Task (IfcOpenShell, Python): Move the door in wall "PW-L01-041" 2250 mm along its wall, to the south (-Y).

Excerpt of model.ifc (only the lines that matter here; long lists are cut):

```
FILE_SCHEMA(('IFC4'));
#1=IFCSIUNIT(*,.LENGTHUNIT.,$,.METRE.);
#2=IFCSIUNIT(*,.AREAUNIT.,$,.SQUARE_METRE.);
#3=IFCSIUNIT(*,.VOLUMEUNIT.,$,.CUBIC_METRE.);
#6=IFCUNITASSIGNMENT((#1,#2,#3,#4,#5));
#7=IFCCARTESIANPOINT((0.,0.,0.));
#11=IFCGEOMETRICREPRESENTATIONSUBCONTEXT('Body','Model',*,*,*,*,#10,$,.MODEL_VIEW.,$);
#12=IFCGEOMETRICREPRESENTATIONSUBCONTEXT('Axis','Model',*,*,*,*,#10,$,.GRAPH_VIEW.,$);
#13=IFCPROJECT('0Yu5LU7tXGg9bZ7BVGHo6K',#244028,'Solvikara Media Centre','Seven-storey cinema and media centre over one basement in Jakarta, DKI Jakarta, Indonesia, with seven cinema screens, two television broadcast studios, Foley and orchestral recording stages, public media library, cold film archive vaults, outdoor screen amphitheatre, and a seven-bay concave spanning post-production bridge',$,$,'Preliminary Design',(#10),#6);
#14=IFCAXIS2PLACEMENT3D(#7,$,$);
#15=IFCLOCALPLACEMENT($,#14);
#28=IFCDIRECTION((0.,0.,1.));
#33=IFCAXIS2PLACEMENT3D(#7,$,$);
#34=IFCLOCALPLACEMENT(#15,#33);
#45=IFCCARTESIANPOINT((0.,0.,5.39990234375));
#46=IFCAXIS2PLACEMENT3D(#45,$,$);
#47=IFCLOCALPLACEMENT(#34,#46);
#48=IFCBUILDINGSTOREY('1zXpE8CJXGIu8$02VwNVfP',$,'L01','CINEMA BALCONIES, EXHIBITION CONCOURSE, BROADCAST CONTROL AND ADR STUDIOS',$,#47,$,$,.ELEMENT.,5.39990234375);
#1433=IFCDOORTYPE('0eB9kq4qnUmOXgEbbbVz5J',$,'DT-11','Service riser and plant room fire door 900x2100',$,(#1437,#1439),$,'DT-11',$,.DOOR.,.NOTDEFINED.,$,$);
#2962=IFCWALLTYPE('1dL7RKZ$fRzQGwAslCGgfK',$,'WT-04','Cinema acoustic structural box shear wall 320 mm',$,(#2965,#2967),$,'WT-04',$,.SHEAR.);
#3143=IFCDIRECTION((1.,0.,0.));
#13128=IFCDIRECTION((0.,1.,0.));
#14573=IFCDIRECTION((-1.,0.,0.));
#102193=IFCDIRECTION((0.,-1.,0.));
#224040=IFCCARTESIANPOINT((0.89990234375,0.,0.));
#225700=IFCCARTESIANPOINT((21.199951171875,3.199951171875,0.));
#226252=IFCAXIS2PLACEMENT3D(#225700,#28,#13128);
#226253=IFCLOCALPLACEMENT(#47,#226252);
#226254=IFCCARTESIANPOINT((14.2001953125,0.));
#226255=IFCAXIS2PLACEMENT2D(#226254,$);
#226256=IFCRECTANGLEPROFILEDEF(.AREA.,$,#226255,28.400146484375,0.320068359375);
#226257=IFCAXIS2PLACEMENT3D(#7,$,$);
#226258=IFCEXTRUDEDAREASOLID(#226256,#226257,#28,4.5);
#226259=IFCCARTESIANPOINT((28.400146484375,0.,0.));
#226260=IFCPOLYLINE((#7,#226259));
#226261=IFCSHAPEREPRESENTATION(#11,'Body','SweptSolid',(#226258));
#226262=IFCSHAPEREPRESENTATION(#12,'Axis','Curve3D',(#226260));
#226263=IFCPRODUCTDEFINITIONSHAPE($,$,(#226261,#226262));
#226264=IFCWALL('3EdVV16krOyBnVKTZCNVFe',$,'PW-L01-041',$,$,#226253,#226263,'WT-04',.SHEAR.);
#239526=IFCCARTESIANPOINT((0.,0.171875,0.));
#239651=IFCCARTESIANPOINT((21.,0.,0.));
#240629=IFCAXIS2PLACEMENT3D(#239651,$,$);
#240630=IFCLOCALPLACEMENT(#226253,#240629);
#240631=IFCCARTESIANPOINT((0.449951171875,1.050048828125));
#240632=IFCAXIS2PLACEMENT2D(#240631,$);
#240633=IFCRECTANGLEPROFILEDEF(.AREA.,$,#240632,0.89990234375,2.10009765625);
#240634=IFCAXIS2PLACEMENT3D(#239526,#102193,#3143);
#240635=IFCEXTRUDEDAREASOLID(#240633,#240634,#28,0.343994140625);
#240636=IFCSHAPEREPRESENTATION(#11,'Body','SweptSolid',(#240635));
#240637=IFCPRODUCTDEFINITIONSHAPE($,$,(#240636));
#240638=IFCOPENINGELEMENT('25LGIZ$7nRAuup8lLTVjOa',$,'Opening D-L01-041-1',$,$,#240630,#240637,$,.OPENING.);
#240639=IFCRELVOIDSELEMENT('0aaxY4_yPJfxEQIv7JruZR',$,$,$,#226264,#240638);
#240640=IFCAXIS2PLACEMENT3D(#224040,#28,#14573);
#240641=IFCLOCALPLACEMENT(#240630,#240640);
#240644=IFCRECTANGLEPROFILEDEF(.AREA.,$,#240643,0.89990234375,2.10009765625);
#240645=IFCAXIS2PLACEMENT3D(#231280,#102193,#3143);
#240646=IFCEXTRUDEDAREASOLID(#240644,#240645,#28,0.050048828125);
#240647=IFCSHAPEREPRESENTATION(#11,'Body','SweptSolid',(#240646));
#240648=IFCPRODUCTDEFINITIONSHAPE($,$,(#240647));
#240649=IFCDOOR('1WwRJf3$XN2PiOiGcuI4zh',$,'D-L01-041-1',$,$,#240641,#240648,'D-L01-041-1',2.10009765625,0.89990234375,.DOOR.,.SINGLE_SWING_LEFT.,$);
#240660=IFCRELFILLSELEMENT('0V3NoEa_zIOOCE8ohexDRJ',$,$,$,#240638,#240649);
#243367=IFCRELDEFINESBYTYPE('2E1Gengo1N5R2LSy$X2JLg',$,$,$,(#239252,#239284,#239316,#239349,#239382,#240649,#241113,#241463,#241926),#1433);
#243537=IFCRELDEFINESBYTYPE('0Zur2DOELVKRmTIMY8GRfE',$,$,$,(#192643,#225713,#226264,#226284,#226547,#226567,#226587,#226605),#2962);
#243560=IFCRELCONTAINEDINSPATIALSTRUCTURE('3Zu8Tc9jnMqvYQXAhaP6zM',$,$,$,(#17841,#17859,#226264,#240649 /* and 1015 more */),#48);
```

```python
import ifcopenshell
import ifcopenshell.api.geometry
import ifcopenshell.util.placement

model = ifcopenshell.open("model.ifc")

door = model.by_guid("1WwRJf3$XN2PiOiGcuI4zh")
opening = door.FillsVoids[0].RelatingOpeningElement
wall = opening.VoidsElements[0].RelatingBuildingElement

wall_matrix = ifcopenshell.util.placement.get_local_placement(wall.ObjectPlacement)
shift = wall_matrix[:3, 0] * -2.25
before = ifcopenshell.util.placement.get_local_placement(door.ObjectPlacement)[:3, 3].copy()

# The door is placed relative to its opening, so it follows when the opening moves.
matrix = ifcopenshell.util.placement.get_local_placement(opening.ObjectPlacement)
matrix[:3, 3] += shift
ifcopenshell.api.geometry.edit_object_placement(
    model, product=opening, matrix=matrix, is_si=False, should_transform_children=True
)

after = ifcopenshell.util.placement.get_local_placement(door.ObjectPlacement)[:3, 3]
print("door moved by", (after - before).round(3) + 0.0)

model.write("model_updated.ifc")
```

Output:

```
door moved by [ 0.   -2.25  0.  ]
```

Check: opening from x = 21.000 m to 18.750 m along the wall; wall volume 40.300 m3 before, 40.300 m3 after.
